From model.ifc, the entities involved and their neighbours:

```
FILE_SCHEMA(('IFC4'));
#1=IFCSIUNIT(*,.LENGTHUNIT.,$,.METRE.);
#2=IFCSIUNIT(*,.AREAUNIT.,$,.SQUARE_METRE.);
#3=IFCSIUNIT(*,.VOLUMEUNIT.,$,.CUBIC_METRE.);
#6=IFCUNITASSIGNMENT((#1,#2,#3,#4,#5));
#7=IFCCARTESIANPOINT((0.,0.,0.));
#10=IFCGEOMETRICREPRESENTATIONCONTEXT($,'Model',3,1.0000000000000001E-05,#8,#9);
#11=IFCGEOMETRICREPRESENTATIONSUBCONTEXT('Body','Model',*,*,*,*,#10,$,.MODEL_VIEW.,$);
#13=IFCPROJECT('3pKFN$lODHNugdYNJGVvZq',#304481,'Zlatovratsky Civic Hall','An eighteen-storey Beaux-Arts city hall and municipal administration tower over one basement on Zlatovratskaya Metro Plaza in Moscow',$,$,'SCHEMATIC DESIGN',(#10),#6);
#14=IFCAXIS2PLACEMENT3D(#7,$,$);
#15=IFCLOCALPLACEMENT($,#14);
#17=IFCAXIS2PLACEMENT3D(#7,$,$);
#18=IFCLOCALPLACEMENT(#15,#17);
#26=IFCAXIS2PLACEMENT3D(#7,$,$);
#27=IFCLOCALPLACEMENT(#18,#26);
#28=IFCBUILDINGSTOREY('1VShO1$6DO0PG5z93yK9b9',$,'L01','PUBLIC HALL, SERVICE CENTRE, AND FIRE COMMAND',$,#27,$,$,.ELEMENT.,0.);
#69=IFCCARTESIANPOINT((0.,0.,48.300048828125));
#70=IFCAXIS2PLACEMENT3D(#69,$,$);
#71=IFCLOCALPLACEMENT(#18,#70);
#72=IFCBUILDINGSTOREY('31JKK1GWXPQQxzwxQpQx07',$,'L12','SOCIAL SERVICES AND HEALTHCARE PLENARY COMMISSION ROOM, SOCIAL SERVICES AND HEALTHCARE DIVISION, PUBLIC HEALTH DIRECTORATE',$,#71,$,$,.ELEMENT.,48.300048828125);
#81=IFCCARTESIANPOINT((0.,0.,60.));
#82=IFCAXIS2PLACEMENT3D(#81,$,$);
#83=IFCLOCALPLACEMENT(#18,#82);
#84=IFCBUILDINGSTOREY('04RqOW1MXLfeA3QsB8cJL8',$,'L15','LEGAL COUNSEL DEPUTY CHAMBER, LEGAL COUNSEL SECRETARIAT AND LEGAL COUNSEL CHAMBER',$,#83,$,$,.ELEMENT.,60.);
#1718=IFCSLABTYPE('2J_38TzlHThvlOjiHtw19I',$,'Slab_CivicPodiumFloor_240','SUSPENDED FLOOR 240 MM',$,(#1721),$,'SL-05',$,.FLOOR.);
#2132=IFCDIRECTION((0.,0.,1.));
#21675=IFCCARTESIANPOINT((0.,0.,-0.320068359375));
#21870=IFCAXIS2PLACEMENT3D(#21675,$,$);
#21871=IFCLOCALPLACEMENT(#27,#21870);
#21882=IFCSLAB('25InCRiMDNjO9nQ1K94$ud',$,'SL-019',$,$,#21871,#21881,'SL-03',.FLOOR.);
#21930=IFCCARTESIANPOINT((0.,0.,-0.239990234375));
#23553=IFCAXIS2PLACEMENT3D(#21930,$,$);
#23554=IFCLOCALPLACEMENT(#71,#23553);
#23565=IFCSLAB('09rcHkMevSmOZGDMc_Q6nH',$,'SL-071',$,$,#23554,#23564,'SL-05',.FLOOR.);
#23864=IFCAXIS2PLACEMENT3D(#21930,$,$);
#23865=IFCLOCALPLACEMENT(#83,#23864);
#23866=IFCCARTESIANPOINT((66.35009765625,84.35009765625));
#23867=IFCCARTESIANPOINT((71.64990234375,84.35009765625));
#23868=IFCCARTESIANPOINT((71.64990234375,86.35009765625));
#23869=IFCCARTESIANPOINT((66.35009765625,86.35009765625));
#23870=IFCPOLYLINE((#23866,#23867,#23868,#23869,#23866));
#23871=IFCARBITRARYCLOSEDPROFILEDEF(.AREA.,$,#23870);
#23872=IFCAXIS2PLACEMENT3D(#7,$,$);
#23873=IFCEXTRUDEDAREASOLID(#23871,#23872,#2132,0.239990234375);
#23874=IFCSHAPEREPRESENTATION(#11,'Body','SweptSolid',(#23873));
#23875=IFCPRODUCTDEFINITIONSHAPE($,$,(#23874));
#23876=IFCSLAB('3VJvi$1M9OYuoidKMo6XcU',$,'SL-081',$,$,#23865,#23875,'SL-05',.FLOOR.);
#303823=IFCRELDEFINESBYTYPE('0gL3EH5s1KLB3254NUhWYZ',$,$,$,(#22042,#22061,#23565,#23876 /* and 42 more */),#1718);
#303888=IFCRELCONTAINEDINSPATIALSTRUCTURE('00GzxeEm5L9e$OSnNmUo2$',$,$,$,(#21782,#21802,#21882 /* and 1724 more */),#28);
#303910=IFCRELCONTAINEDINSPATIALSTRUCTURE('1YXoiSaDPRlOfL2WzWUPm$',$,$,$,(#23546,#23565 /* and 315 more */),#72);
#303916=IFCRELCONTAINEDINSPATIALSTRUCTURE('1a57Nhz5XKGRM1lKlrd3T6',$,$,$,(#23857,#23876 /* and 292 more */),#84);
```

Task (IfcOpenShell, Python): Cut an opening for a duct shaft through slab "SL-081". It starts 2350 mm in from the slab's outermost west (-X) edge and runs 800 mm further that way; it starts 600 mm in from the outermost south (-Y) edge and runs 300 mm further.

```python
import numpy as np
import ifcopenshell
import ifcopenshell.api.feature
import ifcopenshell.api.geometry
import ifcopenshell.api.root
import ifcopenshell.geom
import ifcopenshell.util.placement
import ifcopenshell.util.representation
import ifcopenshell.util.shape
import ifcopenshell.util.unit

model = ifcopenshell.open("model.ifc")
unit_scale = ifcopenshell.util.unit.calculate_unit_scale(model)
settings = ifcopenshell.geom.settings()


def volume(element):
    """Net volume in cubic metres, openings subtracted."""
    shape = ifcopenshell.geom.create_shape(settings, element)
    return ifcopenshell.util.shape.get_volume(shape.geometry)


slab = model.by_guid("3VJvi$1M9OYuoidKMo6XcU")
before = volume(slab)

# Extent in the slab's own axes, in metres. The edges named are its -X and -Y sides.
slab_shape = ifcopenshell.geom.create_shape(settings, slab)
vertices = ifcopenshell.util.shape.get_vertices(slab_shape.geometry)
x_min, y_min, bottom = vertices.min(axis=0)
top = vertices[:, 2].max()

opening = ifcopenshell.api.root.create_entity(model, ifc_class="IfcOpeningElement", name="Duct shaft opening", predefined_type="OPENING")
context = ifcopenshell.util.representation.get_context(model, "Model", "Body", "MODEL_VIEW")
width, depth = 0.8, 0.3
outline = [(0.0, 0.0), (width, 0.0), (width, depth), (0.0, depth), (0.0, 0.0)]
# Overshoot both faces by 50 mm so the cut is clean.
shape = ifcopenshell.api.geometry.add_slab_representation(
    model, context=context, depth=top - bottom + 0.1, polyline=outline
)
ifcopenshell.api.geometry.assign_representation(model, product=opening, representation=shape)

matrix = ifcopenshell.util.placement.get_local_placement(slab.ObjectPlacement)
matrix[:, 3] = matrix @ np.append(np.array([x_min + 2.35, y_min + 0.6, bottom - 0.05]) / unit_scale, 1.0)
ifcopenshell.api.geometry.edit_object_placement(model, product=opening, matrix=matrix, is_si=False)
ifcopenshell.api.feature.add_feature(model, feature=opening, element=slab)

after = volume(slab)

print(f"slab volume {before:.3f} -> {after:.3f} m3")

model.write("model_v2.ifc")
```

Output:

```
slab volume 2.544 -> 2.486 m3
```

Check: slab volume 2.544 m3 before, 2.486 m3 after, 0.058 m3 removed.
